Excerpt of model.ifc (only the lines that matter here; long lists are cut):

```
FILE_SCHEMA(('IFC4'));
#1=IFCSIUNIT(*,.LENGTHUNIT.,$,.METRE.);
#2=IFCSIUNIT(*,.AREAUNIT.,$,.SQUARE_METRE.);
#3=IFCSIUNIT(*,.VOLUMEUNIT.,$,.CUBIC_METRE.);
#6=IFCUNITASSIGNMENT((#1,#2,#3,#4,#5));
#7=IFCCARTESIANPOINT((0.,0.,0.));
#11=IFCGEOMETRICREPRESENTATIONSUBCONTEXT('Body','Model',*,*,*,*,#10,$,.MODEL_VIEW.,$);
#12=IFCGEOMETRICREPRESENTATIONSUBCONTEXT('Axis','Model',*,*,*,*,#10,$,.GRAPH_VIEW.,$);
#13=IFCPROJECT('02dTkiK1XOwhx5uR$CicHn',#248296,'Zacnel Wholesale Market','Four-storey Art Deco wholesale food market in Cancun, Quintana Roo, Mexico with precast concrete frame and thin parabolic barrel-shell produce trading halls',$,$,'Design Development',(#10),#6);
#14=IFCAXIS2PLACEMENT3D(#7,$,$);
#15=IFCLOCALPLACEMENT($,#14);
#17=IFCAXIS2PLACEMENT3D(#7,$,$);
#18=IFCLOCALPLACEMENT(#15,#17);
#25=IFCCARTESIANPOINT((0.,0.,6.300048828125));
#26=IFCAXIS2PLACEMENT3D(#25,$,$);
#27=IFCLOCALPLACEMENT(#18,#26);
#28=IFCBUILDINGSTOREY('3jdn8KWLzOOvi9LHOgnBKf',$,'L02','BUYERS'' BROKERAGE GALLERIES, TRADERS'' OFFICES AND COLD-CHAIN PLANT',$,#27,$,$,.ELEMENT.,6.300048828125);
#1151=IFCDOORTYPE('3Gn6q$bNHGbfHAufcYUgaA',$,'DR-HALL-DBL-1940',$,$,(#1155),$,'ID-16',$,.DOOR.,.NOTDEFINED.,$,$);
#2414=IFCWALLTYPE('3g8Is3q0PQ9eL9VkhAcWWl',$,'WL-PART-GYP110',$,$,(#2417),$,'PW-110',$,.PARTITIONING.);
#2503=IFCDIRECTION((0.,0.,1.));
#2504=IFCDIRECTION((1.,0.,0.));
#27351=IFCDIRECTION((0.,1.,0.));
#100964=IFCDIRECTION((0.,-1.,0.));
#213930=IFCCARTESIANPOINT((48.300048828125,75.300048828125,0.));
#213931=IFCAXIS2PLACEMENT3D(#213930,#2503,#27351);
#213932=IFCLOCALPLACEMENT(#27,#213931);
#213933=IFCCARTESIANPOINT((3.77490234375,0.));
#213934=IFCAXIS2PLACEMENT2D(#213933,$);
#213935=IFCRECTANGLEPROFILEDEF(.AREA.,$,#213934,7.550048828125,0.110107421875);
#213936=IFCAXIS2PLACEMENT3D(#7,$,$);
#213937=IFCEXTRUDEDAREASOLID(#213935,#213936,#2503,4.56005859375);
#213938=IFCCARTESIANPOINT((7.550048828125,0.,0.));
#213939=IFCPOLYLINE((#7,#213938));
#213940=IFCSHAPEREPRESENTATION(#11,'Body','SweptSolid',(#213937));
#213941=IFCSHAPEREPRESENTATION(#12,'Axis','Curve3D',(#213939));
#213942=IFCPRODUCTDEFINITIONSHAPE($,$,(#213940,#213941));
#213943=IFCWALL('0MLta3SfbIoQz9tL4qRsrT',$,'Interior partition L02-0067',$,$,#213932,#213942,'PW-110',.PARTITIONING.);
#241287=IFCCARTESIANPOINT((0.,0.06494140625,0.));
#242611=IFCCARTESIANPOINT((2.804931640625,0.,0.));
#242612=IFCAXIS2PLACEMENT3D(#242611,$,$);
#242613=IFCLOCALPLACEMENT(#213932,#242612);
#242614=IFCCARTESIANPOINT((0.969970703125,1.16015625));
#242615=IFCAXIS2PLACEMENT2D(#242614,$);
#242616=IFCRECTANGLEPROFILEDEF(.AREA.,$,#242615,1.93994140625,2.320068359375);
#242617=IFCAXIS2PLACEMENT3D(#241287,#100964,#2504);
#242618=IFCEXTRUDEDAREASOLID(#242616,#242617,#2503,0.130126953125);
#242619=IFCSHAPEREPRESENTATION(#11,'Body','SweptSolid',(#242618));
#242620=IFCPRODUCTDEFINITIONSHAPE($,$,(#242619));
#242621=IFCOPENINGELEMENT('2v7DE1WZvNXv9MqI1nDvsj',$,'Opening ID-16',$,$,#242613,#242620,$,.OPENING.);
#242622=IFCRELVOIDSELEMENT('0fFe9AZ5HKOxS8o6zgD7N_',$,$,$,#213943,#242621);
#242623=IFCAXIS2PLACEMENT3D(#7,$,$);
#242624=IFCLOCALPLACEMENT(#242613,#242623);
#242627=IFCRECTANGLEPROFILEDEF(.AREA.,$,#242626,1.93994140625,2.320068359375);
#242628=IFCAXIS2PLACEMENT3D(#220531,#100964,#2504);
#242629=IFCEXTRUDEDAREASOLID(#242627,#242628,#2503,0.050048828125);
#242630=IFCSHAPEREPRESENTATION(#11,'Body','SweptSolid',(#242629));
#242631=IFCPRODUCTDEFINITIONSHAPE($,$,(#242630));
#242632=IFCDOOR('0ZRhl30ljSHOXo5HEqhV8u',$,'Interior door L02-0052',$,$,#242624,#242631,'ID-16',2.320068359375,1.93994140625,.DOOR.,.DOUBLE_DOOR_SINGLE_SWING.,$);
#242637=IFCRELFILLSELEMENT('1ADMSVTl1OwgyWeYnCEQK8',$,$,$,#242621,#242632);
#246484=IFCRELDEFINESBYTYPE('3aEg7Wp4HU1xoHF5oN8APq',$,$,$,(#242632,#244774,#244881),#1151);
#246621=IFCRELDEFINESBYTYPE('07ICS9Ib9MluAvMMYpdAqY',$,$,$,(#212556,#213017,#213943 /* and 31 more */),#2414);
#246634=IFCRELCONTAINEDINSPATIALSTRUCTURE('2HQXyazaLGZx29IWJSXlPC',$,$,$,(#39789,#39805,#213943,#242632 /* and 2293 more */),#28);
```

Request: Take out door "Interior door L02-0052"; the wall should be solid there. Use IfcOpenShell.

```python
import ifcopenshell
import ifcopenshell.api.feature
import ifcopenshell.api.root
import ifcopenshell.geom
import ifcopenshell.util.shape

model = ifcopenshell.open("model.ifc")
settings = ifcopenshell.geom.settings()


def volume(element):
    """Net volume in cubic metres, openings subtracted."""
    shape = ifcopenshell.geom.create_shape(settings, element)
    return ifcopenshell.util.shape.get_volume(shape.geometry)


door = model.by_guid("0ZRhl30ljSHOXo5HEqhV8u")
opening = door.FillsVoids[0].RelatingOpeningElement
wall = opening.VoidsElements[0].RelatingBuildingElement
before = volume(wall)

ifcopenshell.api.root.remove_product(model, product=door)
ifcopenshell.api.feature.remove_feature(model, feature=opening)

after = volume(wall)

print(f"wall volume {before:.3f} -> {after:.3f} m3")

model.write("model_edited.ifc")
```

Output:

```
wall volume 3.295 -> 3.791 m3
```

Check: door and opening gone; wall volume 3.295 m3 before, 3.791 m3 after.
